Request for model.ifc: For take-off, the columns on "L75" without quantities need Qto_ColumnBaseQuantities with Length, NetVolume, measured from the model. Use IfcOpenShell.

First a look at what the model holds.

```python
import ifcopenshell
import ifcopenshell.util.element
import ifcopenshell.util.unit

model = ifcopenshell.open("model.ifc")
print(model.schema)
for unit_type in ("LENGTHUNIT", "AREAUNIT", "VOLUMEUNIT"):
    print(unit_type, ifcopenshell.util.unit.calculate_unit_scale(model, unit_type))
storey = next(s for s in model.by_type("IfcBuildingStorey") if s.Name == "L75")
columns = [e for e in ifcopenshell.util.element.get_decomposition(storey) if e.is_a("IfcColumn")]
for e in sorted(columns, key=lambda e: e.id()):
    print(e.id(), e.is_a(), e.Name, list(ifcopenshell.util.element.get_psets(e, qtos_only=True)), sep=" | ")
```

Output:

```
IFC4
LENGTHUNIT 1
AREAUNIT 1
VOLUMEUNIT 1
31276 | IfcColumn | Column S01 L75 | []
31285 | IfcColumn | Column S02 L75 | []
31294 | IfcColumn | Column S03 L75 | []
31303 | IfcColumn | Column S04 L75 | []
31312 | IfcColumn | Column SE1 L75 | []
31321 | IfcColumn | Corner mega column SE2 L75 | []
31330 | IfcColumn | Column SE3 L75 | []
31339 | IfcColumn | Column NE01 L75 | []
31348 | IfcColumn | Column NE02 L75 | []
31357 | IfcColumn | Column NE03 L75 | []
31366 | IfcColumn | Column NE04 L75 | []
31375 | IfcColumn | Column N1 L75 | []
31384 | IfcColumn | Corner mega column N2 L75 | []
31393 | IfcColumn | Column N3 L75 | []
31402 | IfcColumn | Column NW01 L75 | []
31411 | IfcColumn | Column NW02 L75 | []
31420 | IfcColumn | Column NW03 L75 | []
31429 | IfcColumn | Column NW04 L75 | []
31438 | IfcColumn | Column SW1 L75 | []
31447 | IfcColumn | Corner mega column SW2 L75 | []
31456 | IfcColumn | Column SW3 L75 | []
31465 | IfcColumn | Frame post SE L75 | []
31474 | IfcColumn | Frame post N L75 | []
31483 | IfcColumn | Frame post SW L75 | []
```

```python
import ifcopenshell
import ifcopenshell.api.pset
import ifcopenshell.geom
import ifcopenshell.util.element
import ifcopenshell.util.shape
import ifcopenshell.util.unit

model = ifcopenshell.open("model.ifc")
unit_scale = ifcopenshell.util.unit.calculate_unit_scale(model)
volume_scale = ifcopenshell.util.unit.calculate_unit_scale(model, "VOLUMEUNIT")
settings = ifcopenshell.geom.settings()

storey = next(s for s in model.by_type("IfcBuildingStorey") if s.Name == "L75")
columns = [e for e in ifcopenshell.util.element.get_decomposition(storey) if e.is_a("IfcColumn")]

for e in sorted(columns, key=lambda e: e.id()):
    if ifcopenshell.util.element.get_psets(e, qtos_only=True, should_inherit=False):
        continue
    # Geometry comes back in metres, in the element's own axes.
    shape = ifcopenshell.geom.create_shape(settings, e)
    values = {
        "Length": ifcopenshell.util.shape.get_z(shape.geometry) / unit_scale,
        "NetVolume": ifcopenshell.util.shape.get_volume(shape.geometry) / volume_scale,
    }
    qto = ifcopenshell.api.pset.add_qto(model, product=e, name="Qto_ColumnBaseQuantities")
    ifcopenshell.api.pset.edit_qto(model, qto=qto, properties=values)
    print(e.id(), {k: round(v, 3) for k, v in values.items()})

model.write("model_rev.ifc")
```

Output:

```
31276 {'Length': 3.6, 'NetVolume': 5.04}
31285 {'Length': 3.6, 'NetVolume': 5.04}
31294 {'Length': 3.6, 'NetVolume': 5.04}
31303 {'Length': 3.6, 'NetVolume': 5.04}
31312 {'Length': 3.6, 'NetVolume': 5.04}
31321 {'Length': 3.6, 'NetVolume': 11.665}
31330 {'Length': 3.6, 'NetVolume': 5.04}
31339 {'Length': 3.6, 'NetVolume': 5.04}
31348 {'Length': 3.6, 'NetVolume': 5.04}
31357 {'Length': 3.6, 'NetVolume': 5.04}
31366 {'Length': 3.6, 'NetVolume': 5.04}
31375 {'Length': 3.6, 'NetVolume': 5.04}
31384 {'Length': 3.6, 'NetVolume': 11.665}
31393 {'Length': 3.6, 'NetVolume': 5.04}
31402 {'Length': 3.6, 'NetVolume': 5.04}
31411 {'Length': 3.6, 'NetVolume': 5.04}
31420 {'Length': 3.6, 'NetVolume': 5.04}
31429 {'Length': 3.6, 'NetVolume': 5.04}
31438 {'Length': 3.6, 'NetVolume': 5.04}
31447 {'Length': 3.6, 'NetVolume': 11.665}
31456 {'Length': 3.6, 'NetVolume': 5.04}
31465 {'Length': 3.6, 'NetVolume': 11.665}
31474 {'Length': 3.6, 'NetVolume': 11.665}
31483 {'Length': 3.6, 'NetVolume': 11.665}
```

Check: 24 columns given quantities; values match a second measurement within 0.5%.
